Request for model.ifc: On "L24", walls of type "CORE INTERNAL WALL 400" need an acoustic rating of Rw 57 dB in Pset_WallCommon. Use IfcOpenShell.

First a look at what the model holds.

```python
import ifcopenshell
import ifcopenshell.util.element

model = ifcopenshell.open("model.ifc")
print(model.schema)
storey = next(s for s in model.by_type("IfcBuildingStorey") if s.Name == "L24")
walls = [e for e in ifcopenshell.util.element.get_decomposition(storey) if e.is_a("IfcWall")]
seen = {}
for e in walls:
    element_type = ifcopenshell.util.element.get_type(e)
    key = (element_type.Name if element_type != e and element_type else None, ifcopenshell.util.element.get_pset(e, "Pset_WallCommon", "AcousticRating"))
    seen[key] = seen.get(key, 0) + 1
for (name, value), count in sorted(seen.items(), key=str):
    print(count, "x", name, "|", value)
```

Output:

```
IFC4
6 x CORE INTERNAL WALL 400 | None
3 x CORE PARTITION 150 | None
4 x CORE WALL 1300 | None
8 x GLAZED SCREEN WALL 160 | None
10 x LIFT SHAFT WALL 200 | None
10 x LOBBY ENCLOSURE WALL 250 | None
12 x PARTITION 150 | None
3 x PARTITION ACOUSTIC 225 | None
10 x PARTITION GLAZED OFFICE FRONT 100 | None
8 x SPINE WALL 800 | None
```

```python
import ifcopenshell
import ifcopenshell.api.pset
import ifcopenshell.util.element

model = ifcopenshell.open("model.ifc")

storey = next(s for s in model.by_type("IfcBuildingStorey") if s.Name == "L24")
walls = [e for e in ifcopenshell.util.element.get_decomposition(storey) if e.is_a("IfcWall")]

count = 0
for e in walls:
    element_type = ifcopenshell.util.element.get_type(e)
    if element_type in (None, e) or element_type.Name != "CORE INTERNAL WALL 400":
        continue
    found = ifcopenshell.util.element.get_pset(e, "Pset_WallCommon", should_inherit=False)
    if found:
        pset = model.by_id(found["id"])
        if len(ifcopenshell.util.element.get_elements_by_pset(pset)) > 1:
            pset = ifcopenshell.api.pset.unshare_pset(model, products=[e], pset=pset)[0]
    else:
        pset = ifcopenshell.api.pset.add_pset(model, product=e, name="Pset_WallCommon")
    ifcopenshell.api.pset.edit_pset(model, pset=pset, properties={"AcousticRating": "Rw 57 dB"})
    count += 1

print(count, "walls updated")

model.write("model_v2.ifc")
```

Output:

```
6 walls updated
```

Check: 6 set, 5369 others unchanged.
